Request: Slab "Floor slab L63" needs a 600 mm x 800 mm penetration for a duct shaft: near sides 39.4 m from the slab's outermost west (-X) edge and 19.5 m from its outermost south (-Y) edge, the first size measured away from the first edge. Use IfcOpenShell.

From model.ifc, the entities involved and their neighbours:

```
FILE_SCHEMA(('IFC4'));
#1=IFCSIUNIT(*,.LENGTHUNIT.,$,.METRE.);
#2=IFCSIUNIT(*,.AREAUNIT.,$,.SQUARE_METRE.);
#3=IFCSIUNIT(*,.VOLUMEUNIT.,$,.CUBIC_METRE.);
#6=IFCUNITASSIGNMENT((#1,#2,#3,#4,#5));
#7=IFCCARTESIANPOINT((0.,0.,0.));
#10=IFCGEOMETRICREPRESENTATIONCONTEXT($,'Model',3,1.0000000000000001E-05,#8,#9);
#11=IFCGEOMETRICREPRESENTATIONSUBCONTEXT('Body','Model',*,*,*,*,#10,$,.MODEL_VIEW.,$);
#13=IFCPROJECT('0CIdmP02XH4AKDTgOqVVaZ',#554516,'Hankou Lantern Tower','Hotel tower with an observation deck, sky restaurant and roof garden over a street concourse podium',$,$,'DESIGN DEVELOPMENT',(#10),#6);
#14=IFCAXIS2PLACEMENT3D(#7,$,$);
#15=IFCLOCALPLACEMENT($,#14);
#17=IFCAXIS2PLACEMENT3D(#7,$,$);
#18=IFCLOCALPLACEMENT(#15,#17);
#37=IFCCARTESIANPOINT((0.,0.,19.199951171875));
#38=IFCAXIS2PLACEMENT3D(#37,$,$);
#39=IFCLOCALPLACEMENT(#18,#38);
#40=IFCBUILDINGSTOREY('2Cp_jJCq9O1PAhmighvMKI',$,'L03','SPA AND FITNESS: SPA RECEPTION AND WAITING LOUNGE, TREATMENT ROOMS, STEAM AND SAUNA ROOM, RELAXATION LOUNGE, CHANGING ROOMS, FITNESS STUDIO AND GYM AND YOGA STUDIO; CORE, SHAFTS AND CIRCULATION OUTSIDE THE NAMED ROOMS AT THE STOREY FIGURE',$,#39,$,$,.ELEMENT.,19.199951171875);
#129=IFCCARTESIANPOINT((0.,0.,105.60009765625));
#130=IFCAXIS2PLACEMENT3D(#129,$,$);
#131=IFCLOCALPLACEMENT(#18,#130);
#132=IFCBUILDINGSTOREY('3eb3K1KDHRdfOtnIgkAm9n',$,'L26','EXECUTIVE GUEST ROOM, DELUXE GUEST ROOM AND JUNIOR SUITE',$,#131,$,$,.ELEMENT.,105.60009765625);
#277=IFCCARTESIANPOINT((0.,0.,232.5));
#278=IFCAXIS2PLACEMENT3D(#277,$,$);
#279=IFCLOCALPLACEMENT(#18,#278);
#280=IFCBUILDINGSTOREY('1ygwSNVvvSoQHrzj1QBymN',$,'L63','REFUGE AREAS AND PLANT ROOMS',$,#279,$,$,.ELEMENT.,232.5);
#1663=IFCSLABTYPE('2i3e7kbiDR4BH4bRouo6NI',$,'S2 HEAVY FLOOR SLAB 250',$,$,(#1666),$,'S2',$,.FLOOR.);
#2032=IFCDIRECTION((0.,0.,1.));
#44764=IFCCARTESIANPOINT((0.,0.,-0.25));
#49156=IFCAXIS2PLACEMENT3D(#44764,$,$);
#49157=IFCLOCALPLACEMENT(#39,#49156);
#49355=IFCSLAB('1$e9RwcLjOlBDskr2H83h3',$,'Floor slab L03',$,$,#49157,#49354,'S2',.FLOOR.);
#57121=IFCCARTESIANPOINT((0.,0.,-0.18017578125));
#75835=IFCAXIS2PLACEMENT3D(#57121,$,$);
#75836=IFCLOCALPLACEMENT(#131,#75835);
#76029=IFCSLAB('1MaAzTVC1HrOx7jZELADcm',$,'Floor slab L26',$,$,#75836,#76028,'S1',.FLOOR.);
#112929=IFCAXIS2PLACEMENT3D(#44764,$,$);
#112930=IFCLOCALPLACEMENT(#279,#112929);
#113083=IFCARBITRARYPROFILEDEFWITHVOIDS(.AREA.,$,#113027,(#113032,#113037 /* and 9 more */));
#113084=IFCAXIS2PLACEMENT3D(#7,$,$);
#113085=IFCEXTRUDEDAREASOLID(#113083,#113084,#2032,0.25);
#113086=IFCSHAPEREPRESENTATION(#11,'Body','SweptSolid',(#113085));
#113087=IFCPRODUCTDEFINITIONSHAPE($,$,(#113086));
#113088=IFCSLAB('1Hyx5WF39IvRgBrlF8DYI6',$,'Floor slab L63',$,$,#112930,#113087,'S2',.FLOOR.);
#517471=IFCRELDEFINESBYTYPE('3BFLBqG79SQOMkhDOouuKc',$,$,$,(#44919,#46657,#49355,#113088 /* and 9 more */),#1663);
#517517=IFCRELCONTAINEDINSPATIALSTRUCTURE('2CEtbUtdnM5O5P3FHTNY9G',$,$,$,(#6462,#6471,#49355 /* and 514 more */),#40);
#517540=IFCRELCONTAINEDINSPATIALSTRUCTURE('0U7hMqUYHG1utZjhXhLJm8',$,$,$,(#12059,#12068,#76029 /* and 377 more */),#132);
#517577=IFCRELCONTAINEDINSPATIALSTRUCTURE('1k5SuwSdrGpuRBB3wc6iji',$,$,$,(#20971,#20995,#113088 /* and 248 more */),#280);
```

```python
import numpy as np
import ifcopenshell
import ifcopenshell.api.feature
import ifcopenshell.api.geometry
import ifcopenshell.api.root
import ifcopenshell.geom
import ifcopenshell.util.placement
import ifcopenshell.util.representation
import ifcopenshell.util.shape
import ifcopenshell.util.unit

model = ifcopenshell.open("model.ifc")
unit_scale = ifcopenshell.util.unit.calculate_unit_scale(model)
settings = ifcopenshell.geom.settings()


def volume(element):
    """Net volume in cubic metres, openings subtracted."""
    shape = ifcopenshell.geom.create_shape(settings, element)
    return ifcopenshell.util.shape.get_volume(shape.geometry)


slab = model.by_guid("1Hyx5WF39IvRgBrlF8DYI6")
before = volume(slab)

# Extent in the slab's own axes, in metres. The edges named are its -X and -Y sides.
slab_shape = ifcopenshell.geom.create_shape(settings, slab)
vertices = ifcopenshell.util.shape.get_vertices(slab_shape.geometry)
x_min, y_min, bottom = vertices.min(axis=0)
top = vertices[:, 2].max()

opening = ifcopenshell.api.root.create_entity(model, ifc_class="IfcOpeningElement", name="Duct shaft opening", predefined_type="OPENING")
context = ifcopenshell.util.representation.get_context(model, "Model", "Body", "MODEL_VIEW")
width, depth = 0.6, 0.8
outline = [(0.0, 0.0), (width, 0.0), (width, depth), (0.0, depth), (0.0, 0.0)]
# Overshoot both faces by 50 mm so the cut is clean.
shape = ifcopenshell.api.geometry.add_slab_representation(
    model, context=context, depth=top - bottom + 0.1, polyline=outline
)
ifcopenshell.api.geometry.assign_representation(model, product=opening, representation=shape)

matrix = ifcopenshell.util.placement.get_local_placement(slab.ObjectPlacement)
matrix[:, 3] = matrix @ np.append(np.array([x_min + 39.4, y_min + 19.5, bottom - 0.05]) / unit_scale, 1.0)
ifcopenshell.api.geometry.edit_object_placement(model, product=opening, matrix=matrix, is_si=False)
ifcopenshell.api.feature.add_feature(model, feature=opening, element=slab)

after = volume(slab)

print(f"slab volume {before:.3f} -> {after:.3f} m3")

model.write("model_v2.ifc")
```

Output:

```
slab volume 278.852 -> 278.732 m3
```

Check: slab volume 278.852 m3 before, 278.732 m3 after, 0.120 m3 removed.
